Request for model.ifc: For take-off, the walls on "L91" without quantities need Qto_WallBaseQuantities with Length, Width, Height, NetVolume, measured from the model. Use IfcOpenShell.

First a look at what the model holds.

```python
import ifcopenshell
import ifcopenshell.util.element
import ifcopenshell.util.unit

model = ifcopenshell.open("model.ifc")
print(model.schema)
for unit_type in ("LENGTHUNIT", "AREAUNIT", "VOLUMEUNIT"):
    print(unit_type, ifcopenshell.util.unit.calculate_unit_scale(model, unit_type))
storey = next(s for s in model.by_type("IfcBuildingStorey") if s.Name == "L91")
walls = [e for e in ifcopenshell.util.element.get_decomposition(storey) if e.is_a("IfcWall")]
for e in sorted(walls, key=lambda e: e.id()):
    print(e.id(), e.is_a(), e.Name, list(ifcopenshell.util.element.get_psets(e, qtos_only=True)), sep=" | ")
```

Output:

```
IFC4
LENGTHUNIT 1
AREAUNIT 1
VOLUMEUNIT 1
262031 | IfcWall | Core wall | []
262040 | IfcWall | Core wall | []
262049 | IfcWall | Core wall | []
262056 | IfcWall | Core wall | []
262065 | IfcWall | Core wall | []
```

```python
import ifcopenshell
import ifcopenshell.api.pset
import ifcopenshell.geom
import ifcopenshell.util.element
import ifcopenshell.util.shape
import ifcopenshell.util.unit

model = ifcopenshell.open("model.ifc")
unit_scale = ifcopenshell.util.unit.calculate_unit_scale(model)
volume_scale = ifcopenshell.util.unit.calculate_unit_scale(model, "VOLUMEUNIT")
settings = ifcopenshell.geom.settings()

storey = next(s for s in model.by_type("IfcBuildingStorey") if s.Name == "L91")
walls = [e for e in ifcopenshell.util.element.get_decomposition(storey) if e.is_a("IfcWall")]

for e in sorted(walls, key=lambda e: e.id()):
    if ifcopenshell.util.element.get_psets(e, qtos_only=True, should_inherit=False):
        continue
    # Geometry comes back in metres, in the element's own axes.
    shape = ifcopenshell.geom.create_shape(settings, e)
    values = {
        "Length": ifcopenshell.util.shape.get_x(shape.geometry) / unit_scale,
        "Width": ifcopenshell.util.shape.get_y(shape.geometry) / unit_scale,
        "Height": ifcopenshell.util.shape.get_z(shape.geometry) / unit_scale,
        "NetVolume": ifcopenshell.util.shape.get_volume(shape.geometry) / volume_scale,
    }
    qto = ifcopenshell.api.pset.add_qto(model, product=e, name="Qto_WallBaseQuantities")
    ifcopenshell.api.pset.edit_qto(model, qto=qto, properties=values)
    print(e.id(), {k: round(v, 3) for k, v in values.items()})

model.write("model_edited.ifc")
```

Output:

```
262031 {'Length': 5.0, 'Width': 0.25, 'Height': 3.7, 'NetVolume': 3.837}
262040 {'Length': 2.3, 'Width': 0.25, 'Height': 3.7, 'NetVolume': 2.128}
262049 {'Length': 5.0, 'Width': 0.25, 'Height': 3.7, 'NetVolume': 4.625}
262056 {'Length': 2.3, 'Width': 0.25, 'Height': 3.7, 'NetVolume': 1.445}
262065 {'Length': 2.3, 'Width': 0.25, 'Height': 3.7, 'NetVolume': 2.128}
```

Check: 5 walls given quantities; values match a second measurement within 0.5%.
